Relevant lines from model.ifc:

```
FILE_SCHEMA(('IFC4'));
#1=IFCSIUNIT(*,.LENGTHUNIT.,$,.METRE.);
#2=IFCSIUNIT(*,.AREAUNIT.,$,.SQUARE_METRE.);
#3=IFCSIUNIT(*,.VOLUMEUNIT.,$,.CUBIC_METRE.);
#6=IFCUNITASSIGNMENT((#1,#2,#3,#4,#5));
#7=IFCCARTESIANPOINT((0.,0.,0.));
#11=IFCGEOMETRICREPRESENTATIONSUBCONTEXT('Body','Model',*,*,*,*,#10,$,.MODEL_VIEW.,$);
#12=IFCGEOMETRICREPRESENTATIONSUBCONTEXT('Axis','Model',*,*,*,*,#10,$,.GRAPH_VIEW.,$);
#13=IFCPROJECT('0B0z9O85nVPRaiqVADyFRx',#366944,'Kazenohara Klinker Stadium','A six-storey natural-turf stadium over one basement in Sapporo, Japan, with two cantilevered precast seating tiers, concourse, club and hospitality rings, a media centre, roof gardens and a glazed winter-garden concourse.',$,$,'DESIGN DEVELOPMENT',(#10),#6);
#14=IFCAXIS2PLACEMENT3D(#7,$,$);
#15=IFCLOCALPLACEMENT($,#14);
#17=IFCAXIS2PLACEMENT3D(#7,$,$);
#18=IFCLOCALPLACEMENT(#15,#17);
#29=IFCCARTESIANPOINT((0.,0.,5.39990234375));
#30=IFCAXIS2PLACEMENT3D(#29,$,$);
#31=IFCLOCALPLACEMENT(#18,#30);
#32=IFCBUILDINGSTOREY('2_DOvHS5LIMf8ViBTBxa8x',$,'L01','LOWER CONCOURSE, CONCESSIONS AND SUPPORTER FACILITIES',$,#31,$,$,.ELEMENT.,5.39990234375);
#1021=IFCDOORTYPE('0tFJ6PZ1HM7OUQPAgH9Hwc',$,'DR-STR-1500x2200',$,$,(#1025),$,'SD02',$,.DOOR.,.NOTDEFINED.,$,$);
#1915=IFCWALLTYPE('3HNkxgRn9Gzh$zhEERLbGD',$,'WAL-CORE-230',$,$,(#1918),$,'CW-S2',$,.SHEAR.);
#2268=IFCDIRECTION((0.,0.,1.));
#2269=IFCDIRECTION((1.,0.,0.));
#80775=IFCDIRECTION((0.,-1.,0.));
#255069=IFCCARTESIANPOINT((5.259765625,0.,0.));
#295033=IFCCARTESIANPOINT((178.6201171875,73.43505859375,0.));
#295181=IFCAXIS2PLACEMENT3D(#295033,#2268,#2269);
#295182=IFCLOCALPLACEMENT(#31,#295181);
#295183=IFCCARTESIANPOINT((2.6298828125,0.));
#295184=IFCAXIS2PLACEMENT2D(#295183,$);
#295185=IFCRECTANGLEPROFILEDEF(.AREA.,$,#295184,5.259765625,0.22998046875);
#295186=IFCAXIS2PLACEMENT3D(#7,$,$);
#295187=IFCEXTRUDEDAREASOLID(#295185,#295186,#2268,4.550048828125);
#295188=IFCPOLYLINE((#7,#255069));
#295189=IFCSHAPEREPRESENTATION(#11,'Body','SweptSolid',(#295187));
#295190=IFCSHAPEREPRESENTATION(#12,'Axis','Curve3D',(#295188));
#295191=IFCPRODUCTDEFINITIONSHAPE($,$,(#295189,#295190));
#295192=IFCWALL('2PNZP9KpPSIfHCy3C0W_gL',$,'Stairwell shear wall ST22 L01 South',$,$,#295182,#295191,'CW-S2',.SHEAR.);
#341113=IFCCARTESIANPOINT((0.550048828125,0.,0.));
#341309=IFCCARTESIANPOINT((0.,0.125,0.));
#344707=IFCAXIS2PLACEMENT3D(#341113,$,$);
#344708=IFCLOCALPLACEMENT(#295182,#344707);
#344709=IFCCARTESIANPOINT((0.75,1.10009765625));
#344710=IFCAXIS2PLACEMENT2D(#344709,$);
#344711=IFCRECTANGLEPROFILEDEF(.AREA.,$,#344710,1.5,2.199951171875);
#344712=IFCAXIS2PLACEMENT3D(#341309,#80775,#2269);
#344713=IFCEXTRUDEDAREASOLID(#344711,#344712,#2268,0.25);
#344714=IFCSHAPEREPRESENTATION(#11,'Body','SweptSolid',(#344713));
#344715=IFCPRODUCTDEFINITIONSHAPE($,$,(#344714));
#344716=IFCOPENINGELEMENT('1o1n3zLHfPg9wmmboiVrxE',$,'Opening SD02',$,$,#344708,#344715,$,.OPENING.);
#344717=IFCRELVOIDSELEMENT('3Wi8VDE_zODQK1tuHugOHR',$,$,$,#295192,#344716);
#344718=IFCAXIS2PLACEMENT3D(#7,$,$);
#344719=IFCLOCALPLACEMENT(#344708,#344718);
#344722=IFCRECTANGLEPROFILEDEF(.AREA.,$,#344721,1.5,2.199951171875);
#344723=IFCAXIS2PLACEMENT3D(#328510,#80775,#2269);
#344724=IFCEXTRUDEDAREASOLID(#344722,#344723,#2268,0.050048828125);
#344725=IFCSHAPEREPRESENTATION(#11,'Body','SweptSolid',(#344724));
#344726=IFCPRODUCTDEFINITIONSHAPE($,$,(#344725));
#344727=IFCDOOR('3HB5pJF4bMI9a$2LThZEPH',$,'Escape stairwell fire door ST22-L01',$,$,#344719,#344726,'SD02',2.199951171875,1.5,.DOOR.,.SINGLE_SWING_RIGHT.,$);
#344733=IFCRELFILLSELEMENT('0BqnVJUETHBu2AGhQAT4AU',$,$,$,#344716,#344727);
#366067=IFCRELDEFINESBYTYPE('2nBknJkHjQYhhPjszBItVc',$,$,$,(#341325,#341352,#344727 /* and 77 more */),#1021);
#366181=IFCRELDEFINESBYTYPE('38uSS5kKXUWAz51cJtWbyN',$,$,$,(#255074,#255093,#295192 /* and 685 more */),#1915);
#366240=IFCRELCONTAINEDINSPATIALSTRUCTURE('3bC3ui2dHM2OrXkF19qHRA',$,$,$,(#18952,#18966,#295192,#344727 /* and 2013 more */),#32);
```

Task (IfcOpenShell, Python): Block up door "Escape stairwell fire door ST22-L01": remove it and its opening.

```python
import ifcopenshell
import ifcopenshell.api.feature
import ifcopenshell.api.root
import ifcopenshell.geom
import ifcopenshell.util.shape

model = ifcopenshell.open("model.ifc")
settings = ifcopenshell.geom.settings()


def volume(element):
    """Net volume in cubic metres, openings subtracted."""
    shape = ifcopenshell.geom.create_shape(settings, element)
    return ifcopenshell.util.shape.get_volume(shape.geometry)


door = model.by_guid("3HB5pJF4bMI9a$2LThZEPH")
opening = door.FillsVoids[0].RelatingOpeningElement
wall = opening.VoidsElements[0].RelatingBuildingElement
before = volume(wall)

ifcopenshell.api.root.remove_product(model, product=door)
ifcopenshell.api.feature.remove_feature(model, feature=opening)

after = volume(wall)

print(f"wall volume {before:.3f} -> {after:.3f} m3")

model.write("model-out.ifc")
```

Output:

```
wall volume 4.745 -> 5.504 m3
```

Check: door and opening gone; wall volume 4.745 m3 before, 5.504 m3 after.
